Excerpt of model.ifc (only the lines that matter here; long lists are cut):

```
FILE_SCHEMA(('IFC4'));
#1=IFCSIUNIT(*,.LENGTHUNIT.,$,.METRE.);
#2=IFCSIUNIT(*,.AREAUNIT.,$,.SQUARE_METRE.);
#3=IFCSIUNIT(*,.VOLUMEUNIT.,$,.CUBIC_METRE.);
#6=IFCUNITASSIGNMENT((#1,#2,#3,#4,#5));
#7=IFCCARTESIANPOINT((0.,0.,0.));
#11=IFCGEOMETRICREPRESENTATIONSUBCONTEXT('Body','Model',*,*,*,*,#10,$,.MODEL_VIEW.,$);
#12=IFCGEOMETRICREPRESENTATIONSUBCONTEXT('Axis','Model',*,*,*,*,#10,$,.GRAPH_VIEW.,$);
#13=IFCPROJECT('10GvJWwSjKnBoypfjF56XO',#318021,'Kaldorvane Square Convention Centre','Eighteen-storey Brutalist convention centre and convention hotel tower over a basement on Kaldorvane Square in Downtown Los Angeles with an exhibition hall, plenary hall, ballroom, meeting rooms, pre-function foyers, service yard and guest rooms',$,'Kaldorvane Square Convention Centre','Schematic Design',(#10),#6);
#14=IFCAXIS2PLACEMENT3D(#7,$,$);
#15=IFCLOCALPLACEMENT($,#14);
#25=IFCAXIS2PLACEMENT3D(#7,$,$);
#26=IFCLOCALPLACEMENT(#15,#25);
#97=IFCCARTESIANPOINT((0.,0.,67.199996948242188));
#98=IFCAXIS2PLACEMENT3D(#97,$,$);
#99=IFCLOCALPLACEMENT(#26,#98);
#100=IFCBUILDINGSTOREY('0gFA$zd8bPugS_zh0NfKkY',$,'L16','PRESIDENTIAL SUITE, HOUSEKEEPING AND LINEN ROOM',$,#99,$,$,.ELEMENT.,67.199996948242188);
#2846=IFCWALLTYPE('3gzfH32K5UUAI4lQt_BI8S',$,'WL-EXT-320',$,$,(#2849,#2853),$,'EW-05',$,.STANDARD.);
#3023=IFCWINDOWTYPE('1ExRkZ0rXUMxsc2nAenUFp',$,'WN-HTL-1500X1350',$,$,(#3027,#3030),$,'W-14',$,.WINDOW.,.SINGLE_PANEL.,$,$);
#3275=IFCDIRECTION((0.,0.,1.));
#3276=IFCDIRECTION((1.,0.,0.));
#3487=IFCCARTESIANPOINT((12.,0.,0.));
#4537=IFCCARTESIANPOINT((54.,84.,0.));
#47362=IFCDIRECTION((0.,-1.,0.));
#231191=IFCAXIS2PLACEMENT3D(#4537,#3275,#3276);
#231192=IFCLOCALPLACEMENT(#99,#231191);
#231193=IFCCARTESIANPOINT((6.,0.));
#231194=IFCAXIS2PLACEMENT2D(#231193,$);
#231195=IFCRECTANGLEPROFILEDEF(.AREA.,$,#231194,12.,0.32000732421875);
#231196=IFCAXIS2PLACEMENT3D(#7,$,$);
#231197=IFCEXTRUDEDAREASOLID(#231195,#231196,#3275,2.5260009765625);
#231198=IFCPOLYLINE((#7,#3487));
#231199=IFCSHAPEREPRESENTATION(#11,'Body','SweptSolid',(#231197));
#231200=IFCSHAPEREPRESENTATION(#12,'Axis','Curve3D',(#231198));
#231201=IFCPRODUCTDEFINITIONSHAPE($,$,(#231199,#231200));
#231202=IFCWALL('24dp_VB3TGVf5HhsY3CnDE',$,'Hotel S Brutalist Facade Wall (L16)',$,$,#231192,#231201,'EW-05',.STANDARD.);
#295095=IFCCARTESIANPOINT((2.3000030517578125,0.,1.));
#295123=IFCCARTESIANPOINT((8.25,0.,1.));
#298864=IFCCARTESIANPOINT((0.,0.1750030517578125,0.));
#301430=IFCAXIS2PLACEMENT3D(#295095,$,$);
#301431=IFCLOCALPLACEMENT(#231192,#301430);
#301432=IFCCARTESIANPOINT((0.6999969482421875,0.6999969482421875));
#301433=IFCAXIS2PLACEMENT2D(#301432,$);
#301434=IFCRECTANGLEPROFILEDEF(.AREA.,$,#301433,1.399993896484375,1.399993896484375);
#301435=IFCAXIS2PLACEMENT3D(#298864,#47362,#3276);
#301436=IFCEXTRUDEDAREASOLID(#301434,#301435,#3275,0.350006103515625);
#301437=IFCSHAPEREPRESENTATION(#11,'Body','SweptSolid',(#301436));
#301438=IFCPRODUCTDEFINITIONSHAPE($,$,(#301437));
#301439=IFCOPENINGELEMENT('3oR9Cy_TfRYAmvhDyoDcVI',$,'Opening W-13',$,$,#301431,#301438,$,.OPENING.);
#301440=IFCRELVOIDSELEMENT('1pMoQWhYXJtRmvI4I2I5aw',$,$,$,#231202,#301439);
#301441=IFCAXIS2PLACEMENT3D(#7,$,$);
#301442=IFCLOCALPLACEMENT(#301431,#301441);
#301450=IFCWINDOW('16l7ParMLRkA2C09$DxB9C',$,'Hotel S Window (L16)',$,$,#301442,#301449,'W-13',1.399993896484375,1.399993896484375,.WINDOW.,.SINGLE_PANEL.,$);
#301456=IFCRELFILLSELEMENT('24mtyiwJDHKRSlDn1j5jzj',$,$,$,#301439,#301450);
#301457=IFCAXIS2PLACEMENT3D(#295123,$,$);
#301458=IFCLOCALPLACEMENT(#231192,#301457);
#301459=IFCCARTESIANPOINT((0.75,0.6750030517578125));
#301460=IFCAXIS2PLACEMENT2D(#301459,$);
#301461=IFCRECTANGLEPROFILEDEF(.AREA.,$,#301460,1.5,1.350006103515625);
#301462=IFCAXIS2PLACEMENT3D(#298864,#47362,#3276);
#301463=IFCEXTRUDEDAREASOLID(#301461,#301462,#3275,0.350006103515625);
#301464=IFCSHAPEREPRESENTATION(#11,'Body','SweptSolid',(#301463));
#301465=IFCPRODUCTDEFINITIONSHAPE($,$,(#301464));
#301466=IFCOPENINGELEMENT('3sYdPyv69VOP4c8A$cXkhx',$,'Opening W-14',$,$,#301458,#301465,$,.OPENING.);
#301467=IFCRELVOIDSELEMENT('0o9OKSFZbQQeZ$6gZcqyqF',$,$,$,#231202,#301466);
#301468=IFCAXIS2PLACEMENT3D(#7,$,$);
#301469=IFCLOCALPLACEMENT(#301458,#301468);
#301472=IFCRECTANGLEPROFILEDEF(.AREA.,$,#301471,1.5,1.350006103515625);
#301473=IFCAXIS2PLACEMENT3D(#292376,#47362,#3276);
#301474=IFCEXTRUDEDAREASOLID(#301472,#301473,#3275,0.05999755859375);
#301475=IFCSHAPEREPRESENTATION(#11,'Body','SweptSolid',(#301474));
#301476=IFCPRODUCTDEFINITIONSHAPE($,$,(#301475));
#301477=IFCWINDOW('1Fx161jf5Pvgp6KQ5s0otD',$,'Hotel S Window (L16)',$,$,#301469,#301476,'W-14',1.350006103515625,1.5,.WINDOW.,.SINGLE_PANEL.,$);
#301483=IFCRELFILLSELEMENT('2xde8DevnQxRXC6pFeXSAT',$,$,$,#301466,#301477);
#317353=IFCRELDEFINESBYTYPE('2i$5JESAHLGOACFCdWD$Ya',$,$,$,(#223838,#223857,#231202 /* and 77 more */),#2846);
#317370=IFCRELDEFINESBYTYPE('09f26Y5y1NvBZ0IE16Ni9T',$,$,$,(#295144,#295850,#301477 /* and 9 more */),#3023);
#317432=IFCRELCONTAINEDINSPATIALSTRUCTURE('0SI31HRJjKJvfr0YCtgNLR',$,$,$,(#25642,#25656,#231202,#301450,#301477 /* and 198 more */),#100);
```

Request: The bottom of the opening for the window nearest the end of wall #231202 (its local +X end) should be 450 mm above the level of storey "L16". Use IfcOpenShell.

```python
import numpy as np
import ifcopenshell
import ifcopenshell.api.geometry
import ifcopenshell.geom
import ifcopenshell.util.element
import ifcopenshell.util.placement
import ifcopenshell.util.shape
import ifcopenshell.util.unit

model = ifcopenshell.open("model.ifc")
unit_scale = ifcopenshell.util.unit.calculate_unit_scale(model)

window = model.by_id(301477)
opening = window.FillsVoids[0].RelatingOpeningElement
storey = ifcopenshell.util.element.get_container(window, ifc_class="IfcBuildingStorey")
level = ifcopenshell.util.placement.get_local_placement(storey.ObjectPlacement)[2, 3]

# The opening's origin need not be at the sill, so measure its lowest point.
shape = ifcopenshell.geom.create_shape(ifcopenshell.geom.settings(), opening)
bottom = ifcopenshell.util.shape.get_shape_bottom_elevation(shape, shape.geometry) / unit_scale
dz = level + 0.45 / unit_scale - bottom

shift = np.array([0.0, 0.0, dz])
# The window is placed relative to its opening, so it follows when the opening moves.
matrix = ifcopenshell.util.placement.get_local_placement(opening.ObjectPlacement)
matrix[:3, 3] += shift
ifcopenshell.api.geometry.edit_object_placement(
    model, product=opening, matrix=matrix, is_si=False, should_transform_children=True
)

print(f"moved by {dz * unit_scale:+.3f} m")

model.write("model_edited.ifc")
```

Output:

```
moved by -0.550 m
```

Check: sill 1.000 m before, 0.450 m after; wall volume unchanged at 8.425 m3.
